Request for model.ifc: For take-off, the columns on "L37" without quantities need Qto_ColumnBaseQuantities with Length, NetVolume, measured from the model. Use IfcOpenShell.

First a look at what the model holds.

```python
import ifcopenshell
import ifcopenshell.util.element
import ifcopenshell.util.unit

model = ifcopenshell.open("model.ifc")
print(model.schema)
for unit_type in ("LENGTHUNIT", "AREAUNIT", "VOLUMEUNIT"):
    print(unit_type, ifcopenshell.util.unit.calculate_unit_scale(model, unit_type))
storey = next(s for s in model.by_type("IfcBuildingStorey") if s.Name == "L37")
columns = [e for e in ifcopenshell.util.element.get_decomposition(storey) if e.is_a("IfcColumn")]
for e in sorted(columns, key=lambda e: e.id()):
    print(e.id(), e.is_a(), e.Name, list(ifcopenshell.util.element.get_psets(e, qtos_only=True)), sep=" | ")
```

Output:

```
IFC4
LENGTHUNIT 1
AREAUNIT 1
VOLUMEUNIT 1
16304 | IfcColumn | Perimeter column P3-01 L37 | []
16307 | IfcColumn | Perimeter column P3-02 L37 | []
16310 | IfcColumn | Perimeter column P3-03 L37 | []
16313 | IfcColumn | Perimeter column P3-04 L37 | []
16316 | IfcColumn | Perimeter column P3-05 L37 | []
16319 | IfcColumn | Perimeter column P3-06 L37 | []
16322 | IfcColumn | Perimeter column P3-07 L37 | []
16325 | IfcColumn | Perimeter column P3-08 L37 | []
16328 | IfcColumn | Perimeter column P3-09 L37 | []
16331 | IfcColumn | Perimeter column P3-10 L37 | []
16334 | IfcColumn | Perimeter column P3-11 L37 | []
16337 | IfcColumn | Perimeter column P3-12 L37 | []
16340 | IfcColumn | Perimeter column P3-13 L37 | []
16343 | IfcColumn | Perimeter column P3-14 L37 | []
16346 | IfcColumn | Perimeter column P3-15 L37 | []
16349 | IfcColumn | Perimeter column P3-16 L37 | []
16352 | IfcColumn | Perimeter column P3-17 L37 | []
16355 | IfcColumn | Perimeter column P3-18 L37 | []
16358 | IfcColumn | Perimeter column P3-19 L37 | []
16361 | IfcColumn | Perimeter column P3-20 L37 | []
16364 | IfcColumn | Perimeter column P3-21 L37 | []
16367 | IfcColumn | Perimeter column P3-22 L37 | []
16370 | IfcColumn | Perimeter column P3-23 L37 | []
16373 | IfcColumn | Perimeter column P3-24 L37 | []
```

```python
import ifcopenshell
import ifcopenshell.api.pset
import ifcopenshell.geom
import ifcopenshell.util.element
import ifcopenshell.util.shape
import ifcopenshell.util.unit

model = ifcopenshell.open("model.ifc")
unit_scale = ifcopenshell.util.unit.calculate_unit_scale(model)
volume_scale = ifcopenshell.util.unit.calculate_unit_scale(model, "VOLUMEUNIT")
settings = ifcopenshell.geom.settings()

storey = next(s for s in model.by_type("IfcBuildingStorey") if s.Name == "L37")
columns = [e for e in ifcopenshell.util.element.get_decomposition(storey) if e.is_a("IfcColumn")]

for e in sorted(columns, key=lambda e: e.id()):
    if ifcopenshell.util.element.get_psets(e, qtos_only=True, should_inherit=False):
        continue
    # Geometry comes back in metres, in the element's own axes.
    shape = ifcopenshell.geom.create_shape(settings, e)
    values = {
        "Length": ifcopenshell.util.shape.get_z(shape.geometry) / unit_scale,
        "NetVolume": ifcopenshell.util.shape.get_volume(shape.geometry) / volume_scale,
    }
    qto = ifcopenshell.api.pset.add_qto(model, product=e, name="Qto_ColumnBaseQuantities")
    ifcopenshell.api.pset.edit_qto(model, qto=qto, properties=values)
    print(e.id(), {k: round(v, 3) for k, v in values.items()})

model.write("model-out.ifc")
```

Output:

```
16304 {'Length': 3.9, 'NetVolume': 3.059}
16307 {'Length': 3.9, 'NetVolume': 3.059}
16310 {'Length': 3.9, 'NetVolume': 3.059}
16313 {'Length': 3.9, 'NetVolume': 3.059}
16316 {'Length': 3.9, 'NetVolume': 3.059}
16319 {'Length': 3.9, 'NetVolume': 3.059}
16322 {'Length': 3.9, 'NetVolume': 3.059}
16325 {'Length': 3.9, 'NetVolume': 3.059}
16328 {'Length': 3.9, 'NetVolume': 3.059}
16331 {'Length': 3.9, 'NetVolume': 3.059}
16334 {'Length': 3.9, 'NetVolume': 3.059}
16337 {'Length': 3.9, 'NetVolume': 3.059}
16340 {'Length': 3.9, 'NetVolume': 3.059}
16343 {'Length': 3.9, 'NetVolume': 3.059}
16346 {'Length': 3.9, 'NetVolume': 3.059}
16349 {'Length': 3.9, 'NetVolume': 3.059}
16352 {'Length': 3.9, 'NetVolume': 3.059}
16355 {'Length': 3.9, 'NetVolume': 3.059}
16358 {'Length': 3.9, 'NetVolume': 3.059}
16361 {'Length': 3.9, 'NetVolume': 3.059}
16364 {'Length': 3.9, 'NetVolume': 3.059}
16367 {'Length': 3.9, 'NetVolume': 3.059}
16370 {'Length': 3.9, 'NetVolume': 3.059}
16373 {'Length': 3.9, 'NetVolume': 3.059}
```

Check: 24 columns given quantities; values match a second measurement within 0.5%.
